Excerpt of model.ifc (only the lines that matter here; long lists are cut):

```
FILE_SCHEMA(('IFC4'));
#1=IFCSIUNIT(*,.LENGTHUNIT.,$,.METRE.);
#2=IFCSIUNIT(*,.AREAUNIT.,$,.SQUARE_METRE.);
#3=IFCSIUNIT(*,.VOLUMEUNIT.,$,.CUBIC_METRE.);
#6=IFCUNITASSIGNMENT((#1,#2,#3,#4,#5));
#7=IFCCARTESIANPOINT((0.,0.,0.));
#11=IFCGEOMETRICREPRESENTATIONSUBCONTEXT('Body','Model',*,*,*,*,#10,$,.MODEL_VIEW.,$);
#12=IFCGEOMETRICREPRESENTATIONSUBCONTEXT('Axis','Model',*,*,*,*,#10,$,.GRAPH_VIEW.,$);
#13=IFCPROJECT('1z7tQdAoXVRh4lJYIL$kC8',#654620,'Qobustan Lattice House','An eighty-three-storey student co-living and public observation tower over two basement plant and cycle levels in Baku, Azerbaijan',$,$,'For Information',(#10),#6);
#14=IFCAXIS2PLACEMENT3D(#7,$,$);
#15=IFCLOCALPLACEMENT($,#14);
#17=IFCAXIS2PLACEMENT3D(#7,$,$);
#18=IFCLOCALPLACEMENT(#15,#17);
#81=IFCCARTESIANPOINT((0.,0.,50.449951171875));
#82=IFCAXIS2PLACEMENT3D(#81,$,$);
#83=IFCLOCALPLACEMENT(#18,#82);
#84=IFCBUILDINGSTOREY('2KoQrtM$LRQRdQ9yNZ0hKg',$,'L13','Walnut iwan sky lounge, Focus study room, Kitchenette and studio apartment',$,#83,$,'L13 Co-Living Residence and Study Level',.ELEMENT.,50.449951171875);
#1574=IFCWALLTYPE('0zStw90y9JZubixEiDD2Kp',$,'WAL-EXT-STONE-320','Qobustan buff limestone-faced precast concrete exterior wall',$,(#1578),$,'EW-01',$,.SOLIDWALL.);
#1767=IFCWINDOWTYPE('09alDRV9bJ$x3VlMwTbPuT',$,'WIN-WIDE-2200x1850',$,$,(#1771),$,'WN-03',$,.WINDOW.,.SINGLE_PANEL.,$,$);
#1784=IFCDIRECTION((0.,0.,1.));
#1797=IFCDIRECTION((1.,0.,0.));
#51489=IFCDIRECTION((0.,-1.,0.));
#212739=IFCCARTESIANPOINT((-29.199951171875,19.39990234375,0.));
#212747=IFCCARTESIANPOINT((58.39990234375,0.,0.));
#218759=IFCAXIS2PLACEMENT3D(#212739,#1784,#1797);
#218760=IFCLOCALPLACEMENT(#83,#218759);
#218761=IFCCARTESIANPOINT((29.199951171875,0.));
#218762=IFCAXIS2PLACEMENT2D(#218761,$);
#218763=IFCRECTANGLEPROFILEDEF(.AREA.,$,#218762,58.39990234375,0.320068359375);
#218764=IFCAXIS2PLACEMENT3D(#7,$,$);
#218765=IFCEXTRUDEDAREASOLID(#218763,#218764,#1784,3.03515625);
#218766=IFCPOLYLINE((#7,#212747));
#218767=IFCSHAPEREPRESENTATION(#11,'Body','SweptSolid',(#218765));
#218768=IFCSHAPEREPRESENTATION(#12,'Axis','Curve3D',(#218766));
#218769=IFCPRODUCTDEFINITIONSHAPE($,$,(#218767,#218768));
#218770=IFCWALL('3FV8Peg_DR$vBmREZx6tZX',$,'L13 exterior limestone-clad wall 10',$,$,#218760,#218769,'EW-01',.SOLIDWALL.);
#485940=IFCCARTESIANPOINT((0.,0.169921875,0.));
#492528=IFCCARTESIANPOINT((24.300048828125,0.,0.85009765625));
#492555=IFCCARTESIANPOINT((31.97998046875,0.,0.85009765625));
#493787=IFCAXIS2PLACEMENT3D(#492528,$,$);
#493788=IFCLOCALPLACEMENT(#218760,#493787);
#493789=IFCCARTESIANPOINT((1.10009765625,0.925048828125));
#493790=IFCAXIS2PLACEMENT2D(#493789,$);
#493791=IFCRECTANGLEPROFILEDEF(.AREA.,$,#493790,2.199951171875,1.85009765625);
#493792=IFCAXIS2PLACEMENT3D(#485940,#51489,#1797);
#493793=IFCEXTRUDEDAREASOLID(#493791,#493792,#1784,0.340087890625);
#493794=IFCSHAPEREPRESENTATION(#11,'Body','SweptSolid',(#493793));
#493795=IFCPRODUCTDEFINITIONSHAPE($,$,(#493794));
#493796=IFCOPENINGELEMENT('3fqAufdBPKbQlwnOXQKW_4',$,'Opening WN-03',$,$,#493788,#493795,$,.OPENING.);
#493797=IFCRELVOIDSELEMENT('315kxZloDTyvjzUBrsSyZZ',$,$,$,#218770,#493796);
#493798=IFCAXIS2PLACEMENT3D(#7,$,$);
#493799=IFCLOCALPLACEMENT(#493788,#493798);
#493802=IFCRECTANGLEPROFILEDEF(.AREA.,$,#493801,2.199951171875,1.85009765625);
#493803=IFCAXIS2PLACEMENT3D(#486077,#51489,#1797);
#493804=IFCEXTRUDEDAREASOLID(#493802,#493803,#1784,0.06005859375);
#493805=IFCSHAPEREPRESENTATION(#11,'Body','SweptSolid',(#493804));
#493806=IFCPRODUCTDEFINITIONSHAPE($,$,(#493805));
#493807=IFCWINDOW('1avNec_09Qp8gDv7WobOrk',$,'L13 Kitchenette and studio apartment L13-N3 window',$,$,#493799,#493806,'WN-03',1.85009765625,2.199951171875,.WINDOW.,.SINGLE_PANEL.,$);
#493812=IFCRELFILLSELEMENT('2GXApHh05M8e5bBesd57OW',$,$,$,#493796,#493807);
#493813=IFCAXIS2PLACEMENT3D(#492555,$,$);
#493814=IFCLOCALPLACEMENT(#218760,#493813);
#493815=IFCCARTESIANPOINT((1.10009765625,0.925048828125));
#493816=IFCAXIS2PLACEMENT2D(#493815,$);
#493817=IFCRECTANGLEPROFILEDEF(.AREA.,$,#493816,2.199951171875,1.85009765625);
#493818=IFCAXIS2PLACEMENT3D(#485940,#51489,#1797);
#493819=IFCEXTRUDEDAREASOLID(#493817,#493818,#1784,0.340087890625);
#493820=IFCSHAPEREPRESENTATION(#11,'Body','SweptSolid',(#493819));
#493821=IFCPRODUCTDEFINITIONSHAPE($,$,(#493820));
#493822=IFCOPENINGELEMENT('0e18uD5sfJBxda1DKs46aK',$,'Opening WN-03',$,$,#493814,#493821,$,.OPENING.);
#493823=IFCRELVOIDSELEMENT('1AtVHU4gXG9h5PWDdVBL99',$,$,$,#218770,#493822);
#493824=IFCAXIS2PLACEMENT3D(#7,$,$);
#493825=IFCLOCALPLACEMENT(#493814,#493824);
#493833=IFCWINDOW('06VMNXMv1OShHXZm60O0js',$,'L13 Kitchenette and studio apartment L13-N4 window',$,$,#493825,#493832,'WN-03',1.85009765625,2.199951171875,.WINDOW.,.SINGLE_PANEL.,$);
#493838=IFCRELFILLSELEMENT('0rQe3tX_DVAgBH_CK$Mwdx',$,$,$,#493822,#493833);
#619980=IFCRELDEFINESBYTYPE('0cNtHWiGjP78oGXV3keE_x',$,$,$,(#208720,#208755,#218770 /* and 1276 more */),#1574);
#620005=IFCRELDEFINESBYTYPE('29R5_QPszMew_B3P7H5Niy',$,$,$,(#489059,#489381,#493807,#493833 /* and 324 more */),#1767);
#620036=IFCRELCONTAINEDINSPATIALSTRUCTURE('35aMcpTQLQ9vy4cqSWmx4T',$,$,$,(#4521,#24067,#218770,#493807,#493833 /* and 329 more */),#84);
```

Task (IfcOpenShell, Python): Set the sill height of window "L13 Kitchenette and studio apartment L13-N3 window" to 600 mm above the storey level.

```python
import numpy as np
import ifcopenshell
import ifcopenshell.api.geometry
import ifcopenshell.geom
import ifcopenshell.util.element
import ifcopenshell.util.placement
import ifcopenshell.util.shape
import ifcopenshell.util.unit

model = ifcopenshell.open("model.ifc")
unit_scale = ifcopenshell.util.unit.calculate_unit_scale(model)

window = model.by_guid("1avNec_09Qp8gDv7WobOrk")
opening = window.FillsVoids[0].RelatingOpeningElement
storey = ifcopenshell.util.element.get_container(window, ifc_class="IfcBuildingStorey")
level = ifcopenshell.util.placement.get_local_placement(storey.ObjectPlacement)[2, 3]

# The opening's origin need not be at the sill, so measure its lowest point.
shape = ifcopenshell.geom.create_shape(ifcopenshell.geom.settings(), opening)
bottom = ifcopenshell.util.shape.get_shape_bottom_elevation(shape, shape.geometry) / unit_scale
dz = level + 0.6 / unit_scale - bottom

shift = np.array([0.0, 0.0, dz])
# The window is placed relative to its opening, so it follows when the opening moves.
matrix = ifcopenshell.util.placement.get_local_placement(opening.ObjectPlacement)
matrix[:3, 3] += shift
ifcopenshell.api.geometry.edit_object_placement(
    model, product=opening, matrix=matrix, is_si=False, should_transform_children=True
)

print(f"moved by {dz * unit_scale:+.3f} m")

model.write("model_updated.ifc")
```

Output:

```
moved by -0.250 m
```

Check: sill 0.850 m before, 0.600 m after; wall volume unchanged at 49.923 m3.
